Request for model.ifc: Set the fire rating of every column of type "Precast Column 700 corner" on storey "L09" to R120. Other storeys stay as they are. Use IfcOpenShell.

First a look at what the model holds.

```python
import ifcopenshell
import ifcopenshell.util.element

model = ifcopenshell.open("model.ifc")
print(model.schema)
storey = next(s for s in model.by_type("IfcBuildingStorey") if s.Name == "L09")
columns = [e for e in ifcopenshell.util.element.get_decomposition(storey) if e.is_a("IfcColumn")]
seen = {}
for e in columns:
    element_type = ifcopenshell.util.element.get_type(e)
    key = (element_type.Name if element_type != e and element_type else None, ifcopenshell.util.element.get_pset(e, "Pset_ColumnCommon", "FireRating"))
    seen[key] = seen.get(key, 0) + 1
for (name, value), count in sorted(seen.items(), key=str):
    print(count, "x", name, "|", value)
```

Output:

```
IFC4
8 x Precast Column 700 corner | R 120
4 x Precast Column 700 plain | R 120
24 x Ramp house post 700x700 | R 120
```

```python
import ifcopenshell
import ifcopenshell.api.pset
import ifcopenshell.util.element

model = ifcopenshell.open("model.ifc")

storey = next(s for s in model.by_type("IfcBuildingStorey") if s.Name == "L09")
columns = [e for e in ifcopenshell.util.element.get_decomposition(storey) if e.is_a("IfcColumn")]

count = 0
for e in columns:
    element_type = ifcopenshell.util.element.get_type(e)
    if element_type in (None, e) or element_type.Name != "Precast Column 700 corner":
        continue
    # add_pset returns the element's existing set when there is one.
    pset = ifcopenshell.api.pset.add_pset(model, product=e, name="Pset_ColumnCommon")
    ifcopenshell.api.pset.edit_pset(model, pset=pset, properties={"FireRating": "R120"})
    count += 1

print(count, "columns updated")

model.write("model_updated.ifc")
```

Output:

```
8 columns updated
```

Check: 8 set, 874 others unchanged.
